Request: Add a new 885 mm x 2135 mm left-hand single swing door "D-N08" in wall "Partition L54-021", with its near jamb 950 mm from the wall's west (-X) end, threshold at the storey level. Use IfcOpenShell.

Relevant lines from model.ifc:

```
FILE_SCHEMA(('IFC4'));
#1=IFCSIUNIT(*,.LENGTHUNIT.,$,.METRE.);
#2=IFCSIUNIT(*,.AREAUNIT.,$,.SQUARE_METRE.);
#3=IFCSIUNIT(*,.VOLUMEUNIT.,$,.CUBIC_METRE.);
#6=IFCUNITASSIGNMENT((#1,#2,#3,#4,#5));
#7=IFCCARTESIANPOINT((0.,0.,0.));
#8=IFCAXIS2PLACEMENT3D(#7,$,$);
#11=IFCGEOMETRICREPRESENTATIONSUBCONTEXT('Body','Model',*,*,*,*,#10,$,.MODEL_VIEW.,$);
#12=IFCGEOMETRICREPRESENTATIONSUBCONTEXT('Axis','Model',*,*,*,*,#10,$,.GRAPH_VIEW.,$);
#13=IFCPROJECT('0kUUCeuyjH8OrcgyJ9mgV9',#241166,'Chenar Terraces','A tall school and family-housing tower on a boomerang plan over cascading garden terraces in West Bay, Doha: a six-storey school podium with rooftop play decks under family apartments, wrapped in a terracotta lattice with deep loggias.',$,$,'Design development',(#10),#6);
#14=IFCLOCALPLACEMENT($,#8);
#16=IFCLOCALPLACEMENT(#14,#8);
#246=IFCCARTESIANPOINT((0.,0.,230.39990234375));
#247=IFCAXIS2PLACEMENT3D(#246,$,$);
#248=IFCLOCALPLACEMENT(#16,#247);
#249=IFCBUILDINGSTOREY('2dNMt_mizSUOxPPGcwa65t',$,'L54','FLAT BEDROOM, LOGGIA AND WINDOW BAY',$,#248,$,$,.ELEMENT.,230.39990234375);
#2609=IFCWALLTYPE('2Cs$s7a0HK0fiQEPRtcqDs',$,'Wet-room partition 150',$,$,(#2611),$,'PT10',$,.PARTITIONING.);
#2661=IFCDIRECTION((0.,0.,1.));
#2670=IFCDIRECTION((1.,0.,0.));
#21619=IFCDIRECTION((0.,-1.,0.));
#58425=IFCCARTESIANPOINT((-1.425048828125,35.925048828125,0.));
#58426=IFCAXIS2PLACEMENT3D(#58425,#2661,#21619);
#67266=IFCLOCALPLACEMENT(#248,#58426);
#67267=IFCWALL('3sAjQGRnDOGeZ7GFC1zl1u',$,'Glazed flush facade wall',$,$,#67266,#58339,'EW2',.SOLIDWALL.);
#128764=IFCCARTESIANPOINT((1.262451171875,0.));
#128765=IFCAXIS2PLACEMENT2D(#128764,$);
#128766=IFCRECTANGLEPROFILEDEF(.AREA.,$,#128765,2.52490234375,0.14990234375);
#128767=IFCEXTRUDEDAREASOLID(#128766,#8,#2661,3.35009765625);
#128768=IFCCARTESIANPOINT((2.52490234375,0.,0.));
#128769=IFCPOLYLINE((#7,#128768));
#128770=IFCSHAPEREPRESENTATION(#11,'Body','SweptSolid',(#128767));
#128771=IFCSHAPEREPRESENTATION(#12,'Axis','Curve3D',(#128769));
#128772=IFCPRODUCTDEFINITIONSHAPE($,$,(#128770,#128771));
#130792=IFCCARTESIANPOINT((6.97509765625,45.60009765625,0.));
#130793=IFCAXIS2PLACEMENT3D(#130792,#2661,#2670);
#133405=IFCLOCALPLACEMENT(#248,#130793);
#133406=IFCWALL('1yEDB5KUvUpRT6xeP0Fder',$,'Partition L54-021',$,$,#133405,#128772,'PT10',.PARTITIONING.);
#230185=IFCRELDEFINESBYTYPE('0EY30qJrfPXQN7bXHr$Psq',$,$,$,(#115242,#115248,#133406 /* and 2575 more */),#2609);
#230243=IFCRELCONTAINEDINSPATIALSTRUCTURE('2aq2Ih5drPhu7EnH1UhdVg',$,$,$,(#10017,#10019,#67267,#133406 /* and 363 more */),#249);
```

```python
import numpy as np
import ifcopenshell
import ifcopenshell.api.feature
import ifcopenshell.api.geometry
import ifcopenshell.api.root
import ifcopenshell.api.spatial
import ifcopenshell.geom
import ifcopenshell.util.element
import ifcopenshell.util.placement
import ifcopenshell.util.representation
import ifcopenshell.util.shape
import ifcopenshell.util.unit

model = ifcopenshell.open("model.ifc")
unit_scale = ifcopenshell.util.unit.calculate_unit_scale(model)
settings = ifcopenshell.geom.settings()


def volume(element):
    """Net volume in cubic metres, openings subtracted."""
    shape = ifcopenshell.geom.create_shape(settings, element)
    return ifcopenshell.util.shape.get_volume(shape.geometry)


wall = model.by_guid("1yEDB5KUvUpRT6xeP0Fder")
storey = ifcopenshell.util.element.get_container(wall, ifc_class="IfcBuildingStorey")
context = ifcopenshell.util.representation.get_context(model, "Model", "Body", "MODEL_VIEW")
before = volume(wall)

width, height, from_end, sill = 0.885, 2.135, 0.95, 0.0  # metres

# The wall runs along its own X axis, and the end named is its -X end.
wall_shape = ifcopenshell.geom.create_shape(settings, wall)
x, y, z = ifcopenshell.util.shape.get_vertices(wall_shape.geometry).T
start = x.min() + from_end
face, thickness = float(y.min()), float(y.max() - y.min())
wall_matrix = ifcopenshell.util.placement.get_local_placement(wall.ObjectPlacement)
level = ifcopenshell.util.placement.get_local_placement(storey.ObjectPlacement)[2, 3]


def in_wall(x, y):
    """Placement at x, y metres in the wall's axes, at sill height."""
    matrix = wall_matrix.copy()
    matrix[:, 3] = wall_matrix @ np.array([x / unit_scale, y / unit_scale, 0.0, 1.0])
    matrix[2, 3] = level + sill / unit_scale
    return matrix


# Opening: a box that overshoots both wall faces by 50 mm.
opening = ifcopenshell.api.root.create_entity(model, ifc_class="IfcOpeningElement", predefined_type="OPENING")
box = ifcopenshell.api.geometry.add_wall_representation(
    model, context=context, length=width, height=height, thickness=thickness + 0.1
)
ifcopenshell.api.geometry.assign_representation(model, product=opening, representation=box)
ifcopenshell.api.geometry.edit_object_placement(model, product=opening, matrix=in_wall(start, face - 0.05), is_si=False)
ifcopenshell.api.feature.add_feature(model, feature=opening, element=wall)

door = ifcopenshell.api.root.create_entity(model, ifc_class="IfcDoor", name="D-N08", predefined_type="DOOR")
door.OverallWidth, door.OverallHeight = width / unit_scale, height / unit_scale
door.OperationType = "SINGLE_SWING_LEFT"
body = ifcopenshell.api.geometry.add_door_representation(
    model,
    context=context,
    overall_width=door.OverallWidth,
    overall_height=door.OverallHeight,
    operation_type="SINGLE_SWING_LEFT",
    lining_properties={"LiningDepth": thickness / unit_scale, "ThresholdDepth": thickness / unit_scale},
)
ifcopenshell.api.geometry.assign_representation(model, product=door, representation=body)
ifcopenshell.api.spatial.assign_container(model, products=[door], relating_structure=storey)
ifcopenshell.api.feature.add_filling(model, opening=opening, element=door)

# The lining spans the wall, so the door starts at the wall face.
ifcopenshell.api.geometry.edit_object_placement(model, product=door, matrix=in_wall(start, face), is_si=False)

after = volume(wall)

print(f"wall volume {before:.3f} -> {after:.3f} m3")

model.write("model_v2.ifc")
```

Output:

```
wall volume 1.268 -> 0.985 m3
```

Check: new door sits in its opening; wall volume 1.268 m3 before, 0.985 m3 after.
